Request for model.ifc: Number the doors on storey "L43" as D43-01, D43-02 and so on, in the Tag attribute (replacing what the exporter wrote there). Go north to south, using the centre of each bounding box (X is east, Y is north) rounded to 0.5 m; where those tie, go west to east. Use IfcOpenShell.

First a look at what the model holds.

```python
import ifcopenshell
import ifcopenshell.util.element
import ifcopenshell.util.placement

model = ifcopenshell.open("model.ifc")
print(model.schema)
storey = next(s for s in model.by_type("IfcBuildingStorey") if s.Name == "L43")
doors = [e for e in ifcopenshell.util.element.get_decomposition(storey) if e.is_a("IfcDoor")]
for e in sorted(doors, key=lambda e: e.id()):
    origin = ifcopenshell.util.placement.get_local_placement(e.ObjectPlacement)[:3, 3]
    print(e.id(), e.Tag, e.Name, origin.round(2) + 0.0, sep=" | ")
```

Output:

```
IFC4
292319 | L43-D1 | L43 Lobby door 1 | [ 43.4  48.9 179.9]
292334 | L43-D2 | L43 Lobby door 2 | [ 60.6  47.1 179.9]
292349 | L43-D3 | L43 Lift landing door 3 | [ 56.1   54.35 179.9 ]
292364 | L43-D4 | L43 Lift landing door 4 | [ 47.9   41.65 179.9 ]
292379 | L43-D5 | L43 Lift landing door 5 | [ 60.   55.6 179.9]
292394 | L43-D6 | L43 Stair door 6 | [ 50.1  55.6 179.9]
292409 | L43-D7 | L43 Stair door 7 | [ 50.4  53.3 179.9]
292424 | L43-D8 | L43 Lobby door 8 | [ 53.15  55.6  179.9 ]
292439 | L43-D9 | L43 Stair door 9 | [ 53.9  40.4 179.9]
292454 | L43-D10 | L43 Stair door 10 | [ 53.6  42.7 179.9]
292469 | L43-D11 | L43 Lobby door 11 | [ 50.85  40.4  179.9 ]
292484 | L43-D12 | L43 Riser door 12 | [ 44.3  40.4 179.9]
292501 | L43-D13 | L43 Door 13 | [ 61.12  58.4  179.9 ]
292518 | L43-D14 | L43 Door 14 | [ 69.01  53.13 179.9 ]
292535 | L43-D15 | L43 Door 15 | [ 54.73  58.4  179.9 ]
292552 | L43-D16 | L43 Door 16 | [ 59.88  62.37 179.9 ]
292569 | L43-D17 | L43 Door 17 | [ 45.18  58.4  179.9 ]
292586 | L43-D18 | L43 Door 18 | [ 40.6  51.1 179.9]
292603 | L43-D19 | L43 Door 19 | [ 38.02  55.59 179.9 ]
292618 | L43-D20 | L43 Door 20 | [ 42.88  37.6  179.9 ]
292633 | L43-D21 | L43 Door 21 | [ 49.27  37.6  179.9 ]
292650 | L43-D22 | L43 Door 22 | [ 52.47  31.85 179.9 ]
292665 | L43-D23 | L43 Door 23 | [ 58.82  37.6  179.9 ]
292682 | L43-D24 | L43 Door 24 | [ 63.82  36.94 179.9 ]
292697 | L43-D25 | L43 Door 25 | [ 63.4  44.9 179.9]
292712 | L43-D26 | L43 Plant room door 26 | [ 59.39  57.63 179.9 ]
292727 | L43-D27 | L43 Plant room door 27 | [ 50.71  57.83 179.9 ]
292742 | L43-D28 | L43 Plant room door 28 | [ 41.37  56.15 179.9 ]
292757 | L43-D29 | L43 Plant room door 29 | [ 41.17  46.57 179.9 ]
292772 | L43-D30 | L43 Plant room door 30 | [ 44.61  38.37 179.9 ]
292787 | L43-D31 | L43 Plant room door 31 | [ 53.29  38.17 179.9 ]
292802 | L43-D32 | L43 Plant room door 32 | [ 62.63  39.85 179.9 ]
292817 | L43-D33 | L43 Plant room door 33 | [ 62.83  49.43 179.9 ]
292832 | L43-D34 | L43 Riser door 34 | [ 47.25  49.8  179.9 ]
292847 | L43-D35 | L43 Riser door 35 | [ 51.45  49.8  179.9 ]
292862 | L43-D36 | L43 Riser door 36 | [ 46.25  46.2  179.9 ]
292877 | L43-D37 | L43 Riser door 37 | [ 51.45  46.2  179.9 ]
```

```python
import ifcopenshell
import ifcopenshell.geom
import ifcopenshell.util.element
import ifcopenshell.util.shape

model = ifcopenshell.open("model.ifc")
settings = ifcopenshell.geom.settings()
settings.set("use-world-coords", True)


def centre(element):
    shape = ifcopenshell.geom.create_shape(settings, element)
    return ifcopenshell.util.shape.get_bbox_centroid(shape.geometry)


storey = next(s for s in model.by_type("IfcBuildingStorey") if s.Name == "L43")
doors = [e for e in ifcopenshell.util.element.get_decomposition(storey) if e.is_a("IfcDoor")]

# Insertion points can sit at a corner or the storey origin, so sort by the geometry (in metres).
centres = {e: centre(e) for e in doors}
doors.sort(key=lambda e: (-round(centres[e][1] / 0.5), centres[e][0]))

for i, e in enumerate(doors, start=1):
    number = f"D43-{i:02d}"
    e.Tag = number
    print(e.id(), number)

model.write("model_updated.ifc")
```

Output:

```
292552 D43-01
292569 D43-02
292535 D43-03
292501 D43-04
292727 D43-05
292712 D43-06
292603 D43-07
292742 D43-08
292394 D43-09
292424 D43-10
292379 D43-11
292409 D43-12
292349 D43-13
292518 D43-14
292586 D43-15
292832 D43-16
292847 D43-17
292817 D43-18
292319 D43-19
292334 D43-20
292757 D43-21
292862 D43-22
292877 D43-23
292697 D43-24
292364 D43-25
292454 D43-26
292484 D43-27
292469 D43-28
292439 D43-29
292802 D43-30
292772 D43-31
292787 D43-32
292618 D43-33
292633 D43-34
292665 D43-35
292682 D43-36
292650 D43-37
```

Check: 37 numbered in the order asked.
